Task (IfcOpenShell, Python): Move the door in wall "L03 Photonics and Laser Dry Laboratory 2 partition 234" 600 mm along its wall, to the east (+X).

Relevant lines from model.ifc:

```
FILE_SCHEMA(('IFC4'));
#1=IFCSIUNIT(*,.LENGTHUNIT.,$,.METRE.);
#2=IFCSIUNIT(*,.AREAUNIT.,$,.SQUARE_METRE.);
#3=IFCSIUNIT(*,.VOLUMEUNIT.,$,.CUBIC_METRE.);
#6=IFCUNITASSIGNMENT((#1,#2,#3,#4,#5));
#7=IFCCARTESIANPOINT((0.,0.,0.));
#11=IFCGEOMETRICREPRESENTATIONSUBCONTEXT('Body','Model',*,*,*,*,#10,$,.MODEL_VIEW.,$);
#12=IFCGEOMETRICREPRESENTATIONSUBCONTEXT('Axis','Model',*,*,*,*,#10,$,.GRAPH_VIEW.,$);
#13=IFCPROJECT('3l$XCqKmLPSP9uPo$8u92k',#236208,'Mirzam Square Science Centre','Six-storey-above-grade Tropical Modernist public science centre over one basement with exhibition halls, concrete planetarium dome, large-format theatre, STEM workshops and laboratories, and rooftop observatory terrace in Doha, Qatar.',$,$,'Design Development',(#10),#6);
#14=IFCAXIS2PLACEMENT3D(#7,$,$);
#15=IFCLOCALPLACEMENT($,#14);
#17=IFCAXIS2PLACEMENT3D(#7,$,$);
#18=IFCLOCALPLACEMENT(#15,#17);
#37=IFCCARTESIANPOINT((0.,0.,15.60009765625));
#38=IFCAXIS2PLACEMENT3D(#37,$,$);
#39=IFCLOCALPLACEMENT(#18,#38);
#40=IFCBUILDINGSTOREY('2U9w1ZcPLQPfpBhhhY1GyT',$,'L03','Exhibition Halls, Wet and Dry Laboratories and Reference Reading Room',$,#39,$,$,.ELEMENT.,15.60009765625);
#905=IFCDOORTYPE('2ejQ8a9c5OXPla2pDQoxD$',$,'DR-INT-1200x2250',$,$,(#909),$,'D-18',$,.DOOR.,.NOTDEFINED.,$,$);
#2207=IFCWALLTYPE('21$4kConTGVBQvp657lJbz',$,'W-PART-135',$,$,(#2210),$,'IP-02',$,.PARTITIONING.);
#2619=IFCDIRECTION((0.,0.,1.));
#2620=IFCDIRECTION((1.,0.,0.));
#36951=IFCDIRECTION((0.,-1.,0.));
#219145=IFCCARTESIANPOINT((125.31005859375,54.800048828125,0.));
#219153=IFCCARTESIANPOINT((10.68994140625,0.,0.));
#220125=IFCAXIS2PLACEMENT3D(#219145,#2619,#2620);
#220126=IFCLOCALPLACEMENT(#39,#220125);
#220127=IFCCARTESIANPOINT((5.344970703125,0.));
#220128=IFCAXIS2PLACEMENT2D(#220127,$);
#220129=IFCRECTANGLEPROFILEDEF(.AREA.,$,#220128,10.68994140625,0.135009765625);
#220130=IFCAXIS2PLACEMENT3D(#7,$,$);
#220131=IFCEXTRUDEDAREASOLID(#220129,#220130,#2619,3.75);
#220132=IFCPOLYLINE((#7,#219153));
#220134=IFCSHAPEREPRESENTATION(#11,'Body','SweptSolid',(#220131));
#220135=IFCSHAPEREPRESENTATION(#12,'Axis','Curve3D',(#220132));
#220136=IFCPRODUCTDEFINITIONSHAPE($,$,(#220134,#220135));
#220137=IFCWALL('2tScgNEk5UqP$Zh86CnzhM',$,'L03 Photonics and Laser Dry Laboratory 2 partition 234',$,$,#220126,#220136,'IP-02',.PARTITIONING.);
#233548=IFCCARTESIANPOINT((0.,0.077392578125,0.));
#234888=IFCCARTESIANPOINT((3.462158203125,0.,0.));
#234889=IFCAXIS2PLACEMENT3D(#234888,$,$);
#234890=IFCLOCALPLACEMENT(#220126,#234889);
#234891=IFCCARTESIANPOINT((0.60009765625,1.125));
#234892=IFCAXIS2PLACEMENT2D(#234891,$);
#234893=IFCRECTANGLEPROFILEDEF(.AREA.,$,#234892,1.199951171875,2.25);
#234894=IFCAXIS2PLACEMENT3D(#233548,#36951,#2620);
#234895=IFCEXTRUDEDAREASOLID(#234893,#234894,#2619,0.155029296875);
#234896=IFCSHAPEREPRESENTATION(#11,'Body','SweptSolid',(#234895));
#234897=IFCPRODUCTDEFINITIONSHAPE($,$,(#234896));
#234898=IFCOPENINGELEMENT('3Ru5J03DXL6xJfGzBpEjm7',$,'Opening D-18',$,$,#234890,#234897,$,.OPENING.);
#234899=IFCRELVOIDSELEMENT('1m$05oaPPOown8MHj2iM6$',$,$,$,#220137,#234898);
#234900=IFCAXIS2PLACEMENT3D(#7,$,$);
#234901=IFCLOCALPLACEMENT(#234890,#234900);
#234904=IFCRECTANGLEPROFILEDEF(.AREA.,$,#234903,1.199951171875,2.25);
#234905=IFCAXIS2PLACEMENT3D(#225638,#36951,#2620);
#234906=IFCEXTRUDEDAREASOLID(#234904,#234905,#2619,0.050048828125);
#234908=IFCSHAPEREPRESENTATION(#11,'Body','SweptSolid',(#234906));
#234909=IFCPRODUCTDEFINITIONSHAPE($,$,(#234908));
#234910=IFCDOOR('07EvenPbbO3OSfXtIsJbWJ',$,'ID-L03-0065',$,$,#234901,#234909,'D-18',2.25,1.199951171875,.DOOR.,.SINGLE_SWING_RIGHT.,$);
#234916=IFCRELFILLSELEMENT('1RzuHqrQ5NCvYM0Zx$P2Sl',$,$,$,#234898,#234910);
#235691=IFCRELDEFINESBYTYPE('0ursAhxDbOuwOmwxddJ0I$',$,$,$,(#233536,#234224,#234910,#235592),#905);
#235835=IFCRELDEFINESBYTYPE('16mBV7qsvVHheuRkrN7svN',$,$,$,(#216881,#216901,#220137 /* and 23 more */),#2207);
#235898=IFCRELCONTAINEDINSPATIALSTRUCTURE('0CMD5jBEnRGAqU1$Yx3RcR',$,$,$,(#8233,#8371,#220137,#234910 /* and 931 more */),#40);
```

```python
import ifcopenshell
import ifcopenshell.api.geometry
import ifcopenshell.util.placement
import ifcopenshell.util.unit

model = ifcopenshell.open("model.ifc")
unit_scale = ifcopenshell.util.unit.calculate_unit_scale(model)

door = model.by_guid("07EvenPbbO3OSfXtIsJbWJ")
opening = door.FillsVoids[0].RelatingOpeningElement
wall = opening.VoidsElements[0].RelatingBuildingElement

wall_matrix = ifcopenshell.util.placement.get_local_placement(wall.ObjectPlacement)
shift = wall_matrix[:3, 0] * 0.6 / unit_scale
before = ifcopenshell.util.placement.get_local_placement(door.ObjectPlacement)[:3, 3].copy()

# The door is placed relative to its opening, so it follows when the opening moves.
matrix = ifcopenshell.util.placement.get_local_placement(opening.ObjectPlacement)
matrix[:3, 3] += shift
ifcopenshell.api.geometry.edit_object_placement(
    model, product=opening, matrix=matrix, is_si=False, should_transform_children=True
)

after = ifcopenshell.util.placement.get_local_placement(door.ObjectPlacement)[:3, 3]
print("door moved by", (after - before).round(3) + 0.0)

model.write("model_rev.ifc")
```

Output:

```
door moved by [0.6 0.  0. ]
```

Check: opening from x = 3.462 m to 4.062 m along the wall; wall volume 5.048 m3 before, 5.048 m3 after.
